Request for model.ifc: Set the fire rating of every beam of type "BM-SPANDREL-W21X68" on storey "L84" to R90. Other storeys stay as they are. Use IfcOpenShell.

First a look at what the model holds.

```python
import ifcopenshell
import ifcopenshell.util.element

model = ifcopenshell.open("model.ifc")
print(model.schema)
storey = next(s for s in model.by_type("IfcBuildingStorey") if s.Name == "L84")
beams = [e for e in ifcopenshell.util.element.get_decomposition(storey) if e.is_a("IfcBeam")]
seen = {}
for e in beams:
    element_type = ifcopenshell.util.element.get_type(e)
    key = (element_type.Name if element_type != e and element_type else None, ifcopenshell.util.element.get_pset(e, "Pset_BeamCommon", "FireRating"))
    seen[key] = seen.get(key, 0) + 1
for (name, value), count in sorted(seen.items(), key=str):
    print(count, "x", name, "|", value)
```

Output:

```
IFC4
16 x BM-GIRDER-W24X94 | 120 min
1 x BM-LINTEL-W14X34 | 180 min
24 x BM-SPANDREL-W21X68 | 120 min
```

```python
import ifcopenshell
import ifcopenshell.api.pset
import ifcopenshell.util.element

model = ifcopenshell.open("model.ifc")

storey = next(s for s in model.by_type("IfcBuildingStorey") if s.Name == "L84")
beams = [e for e in ifcopenshell.util.element.get_decomposition(storey) if e.is_a("IfcBeam")]

count = 0
for e in beams:
    element_type = ifcopenshell.util.element.get_type(e)
    if element_type in (None, e) or element_type.Name != "BM-SPANDREL-W21X68":
        continue
    # add_pset returns the element's existing set when there is one.
    pset = ifcopenshell.api.pset.add_pset(model, product=e, name="Pset_BeamCommon")
    ifcopenshell.api.pset.edit_pset(model, pset=pset, properties={"FireRating": "R90"})
    count += 1

print(count, "beams updated")

model.write("model-out.ifc")
```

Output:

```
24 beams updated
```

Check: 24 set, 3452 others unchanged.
